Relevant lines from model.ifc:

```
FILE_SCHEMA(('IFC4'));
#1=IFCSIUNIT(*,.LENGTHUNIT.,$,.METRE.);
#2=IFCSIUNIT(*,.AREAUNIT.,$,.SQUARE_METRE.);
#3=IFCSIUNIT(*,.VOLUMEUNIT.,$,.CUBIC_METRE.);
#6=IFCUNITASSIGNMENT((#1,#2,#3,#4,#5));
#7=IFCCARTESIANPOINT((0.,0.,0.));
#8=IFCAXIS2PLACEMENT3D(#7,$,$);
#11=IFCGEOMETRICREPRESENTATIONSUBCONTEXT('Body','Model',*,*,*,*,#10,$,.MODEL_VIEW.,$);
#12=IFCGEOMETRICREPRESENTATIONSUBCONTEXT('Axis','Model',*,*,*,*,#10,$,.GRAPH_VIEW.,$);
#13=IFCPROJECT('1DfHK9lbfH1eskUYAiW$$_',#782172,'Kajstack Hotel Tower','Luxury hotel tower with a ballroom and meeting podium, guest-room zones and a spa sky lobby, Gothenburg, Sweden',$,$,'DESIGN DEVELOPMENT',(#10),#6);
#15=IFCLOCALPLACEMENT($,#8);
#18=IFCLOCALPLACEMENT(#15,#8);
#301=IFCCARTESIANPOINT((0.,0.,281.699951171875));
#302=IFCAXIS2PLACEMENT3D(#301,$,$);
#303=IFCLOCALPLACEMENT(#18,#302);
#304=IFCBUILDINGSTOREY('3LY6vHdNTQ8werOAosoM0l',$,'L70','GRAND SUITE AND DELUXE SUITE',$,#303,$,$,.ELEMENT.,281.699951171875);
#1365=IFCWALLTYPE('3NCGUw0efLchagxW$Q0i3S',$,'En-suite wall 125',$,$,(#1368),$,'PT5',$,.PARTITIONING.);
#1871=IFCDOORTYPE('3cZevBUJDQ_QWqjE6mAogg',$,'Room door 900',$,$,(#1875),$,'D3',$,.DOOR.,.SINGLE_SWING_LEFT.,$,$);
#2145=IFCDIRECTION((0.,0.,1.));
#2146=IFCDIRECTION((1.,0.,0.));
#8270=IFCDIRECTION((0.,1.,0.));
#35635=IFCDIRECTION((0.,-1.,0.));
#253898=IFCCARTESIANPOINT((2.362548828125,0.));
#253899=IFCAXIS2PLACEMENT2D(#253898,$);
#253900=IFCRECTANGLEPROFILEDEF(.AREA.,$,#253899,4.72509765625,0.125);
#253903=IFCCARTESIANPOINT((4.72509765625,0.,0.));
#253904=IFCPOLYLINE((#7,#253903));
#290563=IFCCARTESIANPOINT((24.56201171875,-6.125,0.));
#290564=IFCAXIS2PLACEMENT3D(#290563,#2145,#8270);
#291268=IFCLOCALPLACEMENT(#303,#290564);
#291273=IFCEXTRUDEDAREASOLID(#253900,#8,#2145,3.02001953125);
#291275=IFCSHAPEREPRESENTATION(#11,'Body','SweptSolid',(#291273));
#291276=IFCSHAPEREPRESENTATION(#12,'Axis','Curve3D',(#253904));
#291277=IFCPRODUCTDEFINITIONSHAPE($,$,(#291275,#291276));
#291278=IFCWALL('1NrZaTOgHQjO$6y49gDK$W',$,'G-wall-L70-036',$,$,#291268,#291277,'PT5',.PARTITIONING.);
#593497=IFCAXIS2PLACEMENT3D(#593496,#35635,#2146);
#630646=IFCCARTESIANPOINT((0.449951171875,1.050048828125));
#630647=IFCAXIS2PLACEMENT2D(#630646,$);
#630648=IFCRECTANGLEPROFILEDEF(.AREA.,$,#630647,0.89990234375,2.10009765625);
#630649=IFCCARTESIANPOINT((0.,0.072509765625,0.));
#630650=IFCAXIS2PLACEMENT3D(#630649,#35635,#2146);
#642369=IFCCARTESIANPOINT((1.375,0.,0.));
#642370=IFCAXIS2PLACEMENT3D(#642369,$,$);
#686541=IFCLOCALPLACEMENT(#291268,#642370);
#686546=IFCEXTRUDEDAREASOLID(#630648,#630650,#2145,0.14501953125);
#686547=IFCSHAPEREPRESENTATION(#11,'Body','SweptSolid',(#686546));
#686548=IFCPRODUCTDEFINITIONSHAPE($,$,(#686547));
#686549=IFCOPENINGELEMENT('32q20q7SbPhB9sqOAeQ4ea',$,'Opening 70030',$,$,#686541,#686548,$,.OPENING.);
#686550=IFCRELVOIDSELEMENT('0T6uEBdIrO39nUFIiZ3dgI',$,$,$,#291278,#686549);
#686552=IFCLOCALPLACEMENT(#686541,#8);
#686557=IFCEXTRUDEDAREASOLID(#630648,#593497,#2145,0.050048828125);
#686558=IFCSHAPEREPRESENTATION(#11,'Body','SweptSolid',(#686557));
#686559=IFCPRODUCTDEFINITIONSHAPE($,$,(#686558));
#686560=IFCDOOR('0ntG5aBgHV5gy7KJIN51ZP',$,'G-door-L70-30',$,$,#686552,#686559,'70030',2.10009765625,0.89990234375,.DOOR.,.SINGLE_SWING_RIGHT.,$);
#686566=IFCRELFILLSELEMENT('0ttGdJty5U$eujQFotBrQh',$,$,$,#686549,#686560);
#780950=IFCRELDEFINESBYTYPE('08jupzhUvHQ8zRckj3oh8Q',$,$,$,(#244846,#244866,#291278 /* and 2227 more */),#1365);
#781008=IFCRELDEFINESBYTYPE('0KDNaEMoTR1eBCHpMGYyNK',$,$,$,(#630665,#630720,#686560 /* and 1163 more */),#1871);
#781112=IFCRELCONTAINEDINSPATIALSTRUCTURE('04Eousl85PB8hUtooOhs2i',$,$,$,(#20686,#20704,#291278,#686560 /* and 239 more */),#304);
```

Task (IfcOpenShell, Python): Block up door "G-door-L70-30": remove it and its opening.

```python
import ifcopenshell
import ifcopenshell.api.feature
import ifcopenshell.api.root
import ifcopenshell.geom
import ifcopenshell.util.shape

model = ifcopenshell.open("model.ifc")
settings = ifcopenshell.geom.settings()


def volume(element):
    """Net volume in cubic metres, openings subtracted."""
    shape = ifcopenshell.geom.create_shape(settings, element)
    return ifcopenshell.util.shape.get_volume(shape.geometry)


door = model.by_guid("0ntG5aBgHV5gy7KJIN51ZP")
opening = door.FillsVoids[0].RelatingOpeningElement
wall = opening.VoidsElements[0].RelatingBuildingElement
before = volume(wall)

ifcopenshell.api.root.remove_product(model, product=door)
ifcopenshell.api.feature.remove_feature(model, feature=opening)

after = volume(wall)

print(f"wall volume {before:.3f} -> {after:.3f} m3")

model.write("model_rev.ifc")
```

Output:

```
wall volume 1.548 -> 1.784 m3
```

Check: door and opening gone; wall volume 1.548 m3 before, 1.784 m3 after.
